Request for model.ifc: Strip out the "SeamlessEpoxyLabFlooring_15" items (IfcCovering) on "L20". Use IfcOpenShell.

First a look at what the model holds.

```python
import ifcopenshell
import ifcopenshell.util.element

model = ifcopenshell.open("model.ifc")
print(model.schema)
storey = next(s for s in model.by_type("IfcBuildingStorey") if s.Name == "L20")
coverings = [e for e in ifcopenshell.util.element.get_decomposition(storey) if e.is_a("IfcCovering")]
seen = {}
for e in coverings:
    element_type = ifcopenshell.util.element.get_type(e)
    name = element_type.Name if element_type not in (None, e) else None
    seen[name] = seen.get(name, 0) + 1
for name, count in sorted(seen.items(), key=str):
    print(count, "x", name)
```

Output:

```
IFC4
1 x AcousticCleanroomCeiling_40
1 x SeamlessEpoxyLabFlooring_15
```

```python
import ifcopenshell
import ifcopenshell.api.root
import ifcopenshell.util.element

model = ifcopenshell.open("model.ifc")

storey = next(s for s in model.by_type("IfcBuildingStorey") if s.Name == "L20")
coverings = [e for e in ifcopenshell.util.element.get_decomposition(storey) if e.is_a("IfcCovering")]
targets = [e for e in coverings if (t := ifcopenshell.util.element.get_type(e)) not in (None, e) and t.Name == "SeamlessEpoxyLabFlooring_15"]

for e in targets:
    ifcopenshell.api.root.remove_product(model, product=e)
print(len(targets), "removed")

model.write("model-out.ifc")
```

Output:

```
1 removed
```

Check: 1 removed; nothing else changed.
